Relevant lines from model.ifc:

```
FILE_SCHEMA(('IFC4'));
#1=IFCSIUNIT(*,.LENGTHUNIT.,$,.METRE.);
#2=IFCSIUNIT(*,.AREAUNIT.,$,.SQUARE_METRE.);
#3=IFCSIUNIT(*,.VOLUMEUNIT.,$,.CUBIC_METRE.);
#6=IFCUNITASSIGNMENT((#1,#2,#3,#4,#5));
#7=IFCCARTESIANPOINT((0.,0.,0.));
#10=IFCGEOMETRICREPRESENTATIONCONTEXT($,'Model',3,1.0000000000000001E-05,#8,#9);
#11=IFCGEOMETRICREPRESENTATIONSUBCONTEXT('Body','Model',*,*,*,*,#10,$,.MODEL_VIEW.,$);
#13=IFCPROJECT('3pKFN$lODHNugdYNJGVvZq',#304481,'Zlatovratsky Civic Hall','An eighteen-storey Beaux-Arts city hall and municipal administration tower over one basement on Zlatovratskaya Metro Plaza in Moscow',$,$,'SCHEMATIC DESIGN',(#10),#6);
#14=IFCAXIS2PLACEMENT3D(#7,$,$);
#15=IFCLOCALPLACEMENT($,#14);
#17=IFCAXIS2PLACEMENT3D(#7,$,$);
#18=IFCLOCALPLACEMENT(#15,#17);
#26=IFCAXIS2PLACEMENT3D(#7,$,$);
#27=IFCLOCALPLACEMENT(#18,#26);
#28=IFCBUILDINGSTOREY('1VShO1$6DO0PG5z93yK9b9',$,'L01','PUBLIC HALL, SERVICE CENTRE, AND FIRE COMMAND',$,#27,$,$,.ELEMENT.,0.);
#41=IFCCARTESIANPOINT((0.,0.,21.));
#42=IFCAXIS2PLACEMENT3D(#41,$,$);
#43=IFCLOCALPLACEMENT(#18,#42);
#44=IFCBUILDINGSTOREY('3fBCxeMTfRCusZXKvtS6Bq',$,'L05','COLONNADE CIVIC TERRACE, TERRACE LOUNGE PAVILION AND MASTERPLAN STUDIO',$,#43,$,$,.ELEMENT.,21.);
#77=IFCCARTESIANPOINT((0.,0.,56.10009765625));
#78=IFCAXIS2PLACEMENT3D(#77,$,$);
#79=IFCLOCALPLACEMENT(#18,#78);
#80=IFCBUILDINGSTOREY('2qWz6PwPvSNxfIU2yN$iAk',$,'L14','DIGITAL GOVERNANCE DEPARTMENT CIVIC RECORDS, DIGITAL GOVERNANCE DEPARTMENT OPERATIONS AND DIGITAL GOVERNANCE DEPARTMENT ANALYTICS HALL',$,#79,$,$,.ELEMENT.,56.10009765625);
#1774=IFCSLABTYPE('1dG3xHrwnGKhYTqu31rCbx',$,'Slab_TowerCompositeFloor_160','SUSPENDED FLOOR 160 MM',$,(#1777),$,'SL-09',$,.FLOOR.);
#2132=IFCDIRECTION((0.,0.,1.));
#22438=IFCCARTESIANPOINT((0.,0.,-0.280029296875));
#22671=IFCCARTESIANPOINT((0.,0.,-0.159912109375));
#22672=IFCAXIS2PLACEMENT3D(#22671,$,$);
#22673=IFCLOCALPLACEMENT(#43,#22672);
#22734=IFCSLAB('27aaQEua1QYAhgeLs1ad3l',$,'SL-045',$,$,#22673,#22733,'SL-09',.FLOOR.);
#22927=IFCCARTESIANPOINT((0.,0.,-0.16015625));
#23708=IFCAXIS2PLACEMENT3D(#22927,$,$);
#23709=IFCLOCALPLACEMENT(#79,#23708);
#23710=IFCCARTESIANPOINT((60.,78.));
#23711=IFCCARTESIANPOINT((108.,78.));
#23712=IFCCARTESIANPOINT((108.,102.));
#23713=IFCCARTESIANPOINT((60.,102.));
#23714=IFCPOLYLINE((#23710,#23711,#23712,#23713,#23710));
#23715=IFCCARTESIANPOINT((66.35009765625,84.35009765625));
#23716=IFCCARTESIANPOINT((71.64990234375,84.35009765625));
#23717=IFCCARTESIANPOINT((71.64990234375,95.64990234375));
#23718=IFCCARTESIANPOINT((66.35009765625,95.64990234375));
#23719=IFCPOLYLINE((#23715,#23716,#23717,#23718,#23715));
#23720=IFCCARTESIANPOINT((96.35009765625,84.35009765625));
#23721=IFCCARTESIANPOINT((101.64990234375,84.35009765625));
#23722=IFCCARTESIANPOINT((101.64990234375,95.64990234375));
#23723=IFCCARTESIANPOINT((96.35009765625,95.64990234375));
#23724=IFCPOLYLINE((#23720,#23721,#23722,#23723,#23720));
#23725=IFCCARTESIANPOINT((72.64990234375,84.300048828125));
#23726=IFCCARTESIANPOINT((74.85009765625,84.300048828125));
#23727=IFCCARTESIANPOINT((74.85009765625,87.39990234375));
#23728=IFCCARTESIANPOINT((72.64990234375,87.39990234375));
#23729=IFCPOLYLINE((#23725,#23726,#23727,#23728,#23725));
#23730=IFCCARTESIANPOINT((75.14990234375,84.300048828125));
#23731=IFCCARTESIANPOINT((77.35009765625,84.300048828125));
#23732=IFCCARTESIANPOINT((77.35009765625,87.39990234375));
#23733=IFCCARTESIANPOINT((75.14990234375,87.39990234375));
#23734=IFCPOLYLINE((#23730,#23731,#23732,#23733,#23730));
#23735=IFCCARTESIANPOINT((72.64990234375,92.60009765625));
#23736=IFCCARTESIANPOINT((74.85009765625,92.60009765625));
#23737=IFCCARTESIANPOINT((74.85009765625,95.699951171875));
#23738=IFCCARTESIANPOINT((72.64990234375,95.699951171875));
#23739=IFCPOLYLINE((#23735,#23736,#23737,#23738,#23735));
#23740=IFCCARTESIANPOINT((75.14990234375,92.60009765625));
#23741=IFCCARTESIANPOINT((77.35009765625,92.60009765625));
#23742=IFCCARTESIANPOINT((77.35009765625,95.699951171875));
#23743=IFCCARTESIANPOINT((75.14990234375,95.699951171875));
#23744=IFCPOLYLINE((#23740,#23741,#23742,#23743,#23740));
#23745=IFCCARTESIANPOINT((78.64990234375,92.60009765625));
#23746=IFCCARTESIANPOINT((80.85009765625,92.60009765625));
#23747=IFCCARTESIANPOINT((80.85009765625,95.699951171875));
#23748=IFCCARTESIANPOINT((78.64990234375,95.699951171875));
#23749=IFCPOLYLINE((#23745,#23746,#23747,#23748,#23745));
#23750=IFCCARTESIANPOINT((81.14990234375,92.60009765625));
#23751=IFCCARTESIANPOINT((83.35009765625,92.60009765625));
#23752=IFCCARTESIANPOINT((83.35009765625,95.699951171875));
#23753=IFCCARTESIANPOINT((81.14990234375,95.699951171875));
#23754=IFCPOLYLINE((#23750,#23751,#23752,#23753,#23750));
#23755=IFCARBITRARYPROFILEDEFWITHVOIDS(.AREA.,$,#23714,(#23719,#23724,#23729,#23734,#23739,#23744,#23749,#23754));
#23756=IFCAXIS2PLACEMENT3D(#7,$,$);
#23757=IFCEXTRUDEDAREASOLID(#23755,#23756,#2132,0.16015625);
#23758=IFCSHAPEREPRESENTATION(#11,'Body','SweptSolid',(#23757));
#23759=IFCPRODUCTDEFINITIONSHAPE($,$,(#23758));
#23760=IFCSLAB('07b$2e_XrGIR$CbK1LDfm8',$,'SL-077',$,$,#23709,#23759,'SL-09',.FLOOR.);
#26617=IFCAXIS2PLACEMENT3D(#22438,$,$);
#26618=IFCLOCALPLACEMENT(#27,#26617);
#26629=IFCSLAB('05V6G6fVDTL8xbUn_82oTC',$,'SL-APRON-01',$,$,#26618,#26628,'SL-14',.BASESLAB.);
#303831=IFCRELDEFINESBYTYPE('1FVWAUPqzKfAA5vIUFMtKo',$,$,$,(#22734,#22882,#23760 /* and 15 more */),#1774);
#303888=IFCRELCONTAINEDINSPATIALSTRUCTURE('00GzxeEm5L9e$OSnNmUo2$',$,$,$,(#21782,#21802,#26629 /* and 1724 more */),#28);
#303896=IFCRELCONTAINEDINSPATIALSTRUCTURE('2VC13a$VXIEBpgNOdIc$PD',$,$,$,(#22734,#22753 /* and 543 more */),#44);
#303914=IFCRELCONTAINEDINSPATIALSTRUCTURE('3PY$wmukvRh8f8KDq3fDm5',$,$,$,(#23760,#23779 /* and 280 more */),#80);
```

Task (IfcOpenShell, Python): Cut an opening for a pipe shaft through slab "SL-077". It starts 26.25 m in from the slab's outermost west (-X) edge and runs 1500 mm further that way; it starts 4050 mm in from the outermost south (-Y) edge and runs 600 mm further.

```python
import numpy as np
import ifcopenshell
import ifcopenshell.api.feature
import ifcopenshell.api.geometry
import ifcopenshell.api.root
import ifcopenshell.geom
import ifcopenshell.util.placement
import ifcopenshell.util.representation
import ifcopenshell.util.shape
import ifcopenshell.util.unit

model = ifcopenshell.open("model.ifc")
unit_scale = ifcopenshell.util.unit.calculate_unit_scale(model)
settings = ifcopenshell.geom.settings()


def volume(element):
    """Net volume in cubic metres, openings subtracted."""
    shape = ifcopenshell.geom.create_shape(settings, element)
    return ifcopenshell.util.shape.get_volume(shape.geometry)


slab = model.by_id(23760)
before = volume(slab)

# Extent in the slab's own axes, in metres. The edges named are its -X and -Y sides.
slab_shape = ifcopenshell.geom.create_shape(settings, slab)
vertices = ifcopenshell.util.shape.get_vertices(slab_shape.geometry)
x_min, y_min, bottom = vertices.min(axis=0)
top = vertices[:, 2].max()

opening = ifcopenshell.api.root.create_entity(model, ifc_class="IfcOpeningElement", name="Pipe shaft opening", predefined_type="OPENING")
context = ifcopenshell.util.representation.get_context(model, "Model", "Body", "MODEL_VIEW")
width, depth = 1.5, 0.6
outline = [(0.0, 0.0), (width, 0.0), (width, depth), (0.0, depth), (0.0, 0.0)]
# Overshoot both faces by 50 mm so the cut is clean.
shape = ifcopenshell.api.geometry.add_slab_representation(
    model, context=context, depth=top - bottom + 0.1, polyline=outline
)
ifcopenshell.api.geometry.assign_representation(model, product=opening, representation=shape)

matrix = ifcopenshell.util.placement.get_local_placement(slab.ObjectPlacement)
matrix[:, 3] = matrix @ np.append(np.array([x_min + 26.25, y_min + 4.05, bottom - 0.05]) / unit_scale, 1.0)
ifcopenshell.api.geometry.edit_object_placement(model, product=opening, matrix=matrix, is_si=False)
ifcopenshell.api.feature.add_feature(model, feature=opening, element=slab)

after = volume(slab)

print(f"slab volume {before:.3f} -> {after:.3f} m3")

model.write("model_edited.ifc")
```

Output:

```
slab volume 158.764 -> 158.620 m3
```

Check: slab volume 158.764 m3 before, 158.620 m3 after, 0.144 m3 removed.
